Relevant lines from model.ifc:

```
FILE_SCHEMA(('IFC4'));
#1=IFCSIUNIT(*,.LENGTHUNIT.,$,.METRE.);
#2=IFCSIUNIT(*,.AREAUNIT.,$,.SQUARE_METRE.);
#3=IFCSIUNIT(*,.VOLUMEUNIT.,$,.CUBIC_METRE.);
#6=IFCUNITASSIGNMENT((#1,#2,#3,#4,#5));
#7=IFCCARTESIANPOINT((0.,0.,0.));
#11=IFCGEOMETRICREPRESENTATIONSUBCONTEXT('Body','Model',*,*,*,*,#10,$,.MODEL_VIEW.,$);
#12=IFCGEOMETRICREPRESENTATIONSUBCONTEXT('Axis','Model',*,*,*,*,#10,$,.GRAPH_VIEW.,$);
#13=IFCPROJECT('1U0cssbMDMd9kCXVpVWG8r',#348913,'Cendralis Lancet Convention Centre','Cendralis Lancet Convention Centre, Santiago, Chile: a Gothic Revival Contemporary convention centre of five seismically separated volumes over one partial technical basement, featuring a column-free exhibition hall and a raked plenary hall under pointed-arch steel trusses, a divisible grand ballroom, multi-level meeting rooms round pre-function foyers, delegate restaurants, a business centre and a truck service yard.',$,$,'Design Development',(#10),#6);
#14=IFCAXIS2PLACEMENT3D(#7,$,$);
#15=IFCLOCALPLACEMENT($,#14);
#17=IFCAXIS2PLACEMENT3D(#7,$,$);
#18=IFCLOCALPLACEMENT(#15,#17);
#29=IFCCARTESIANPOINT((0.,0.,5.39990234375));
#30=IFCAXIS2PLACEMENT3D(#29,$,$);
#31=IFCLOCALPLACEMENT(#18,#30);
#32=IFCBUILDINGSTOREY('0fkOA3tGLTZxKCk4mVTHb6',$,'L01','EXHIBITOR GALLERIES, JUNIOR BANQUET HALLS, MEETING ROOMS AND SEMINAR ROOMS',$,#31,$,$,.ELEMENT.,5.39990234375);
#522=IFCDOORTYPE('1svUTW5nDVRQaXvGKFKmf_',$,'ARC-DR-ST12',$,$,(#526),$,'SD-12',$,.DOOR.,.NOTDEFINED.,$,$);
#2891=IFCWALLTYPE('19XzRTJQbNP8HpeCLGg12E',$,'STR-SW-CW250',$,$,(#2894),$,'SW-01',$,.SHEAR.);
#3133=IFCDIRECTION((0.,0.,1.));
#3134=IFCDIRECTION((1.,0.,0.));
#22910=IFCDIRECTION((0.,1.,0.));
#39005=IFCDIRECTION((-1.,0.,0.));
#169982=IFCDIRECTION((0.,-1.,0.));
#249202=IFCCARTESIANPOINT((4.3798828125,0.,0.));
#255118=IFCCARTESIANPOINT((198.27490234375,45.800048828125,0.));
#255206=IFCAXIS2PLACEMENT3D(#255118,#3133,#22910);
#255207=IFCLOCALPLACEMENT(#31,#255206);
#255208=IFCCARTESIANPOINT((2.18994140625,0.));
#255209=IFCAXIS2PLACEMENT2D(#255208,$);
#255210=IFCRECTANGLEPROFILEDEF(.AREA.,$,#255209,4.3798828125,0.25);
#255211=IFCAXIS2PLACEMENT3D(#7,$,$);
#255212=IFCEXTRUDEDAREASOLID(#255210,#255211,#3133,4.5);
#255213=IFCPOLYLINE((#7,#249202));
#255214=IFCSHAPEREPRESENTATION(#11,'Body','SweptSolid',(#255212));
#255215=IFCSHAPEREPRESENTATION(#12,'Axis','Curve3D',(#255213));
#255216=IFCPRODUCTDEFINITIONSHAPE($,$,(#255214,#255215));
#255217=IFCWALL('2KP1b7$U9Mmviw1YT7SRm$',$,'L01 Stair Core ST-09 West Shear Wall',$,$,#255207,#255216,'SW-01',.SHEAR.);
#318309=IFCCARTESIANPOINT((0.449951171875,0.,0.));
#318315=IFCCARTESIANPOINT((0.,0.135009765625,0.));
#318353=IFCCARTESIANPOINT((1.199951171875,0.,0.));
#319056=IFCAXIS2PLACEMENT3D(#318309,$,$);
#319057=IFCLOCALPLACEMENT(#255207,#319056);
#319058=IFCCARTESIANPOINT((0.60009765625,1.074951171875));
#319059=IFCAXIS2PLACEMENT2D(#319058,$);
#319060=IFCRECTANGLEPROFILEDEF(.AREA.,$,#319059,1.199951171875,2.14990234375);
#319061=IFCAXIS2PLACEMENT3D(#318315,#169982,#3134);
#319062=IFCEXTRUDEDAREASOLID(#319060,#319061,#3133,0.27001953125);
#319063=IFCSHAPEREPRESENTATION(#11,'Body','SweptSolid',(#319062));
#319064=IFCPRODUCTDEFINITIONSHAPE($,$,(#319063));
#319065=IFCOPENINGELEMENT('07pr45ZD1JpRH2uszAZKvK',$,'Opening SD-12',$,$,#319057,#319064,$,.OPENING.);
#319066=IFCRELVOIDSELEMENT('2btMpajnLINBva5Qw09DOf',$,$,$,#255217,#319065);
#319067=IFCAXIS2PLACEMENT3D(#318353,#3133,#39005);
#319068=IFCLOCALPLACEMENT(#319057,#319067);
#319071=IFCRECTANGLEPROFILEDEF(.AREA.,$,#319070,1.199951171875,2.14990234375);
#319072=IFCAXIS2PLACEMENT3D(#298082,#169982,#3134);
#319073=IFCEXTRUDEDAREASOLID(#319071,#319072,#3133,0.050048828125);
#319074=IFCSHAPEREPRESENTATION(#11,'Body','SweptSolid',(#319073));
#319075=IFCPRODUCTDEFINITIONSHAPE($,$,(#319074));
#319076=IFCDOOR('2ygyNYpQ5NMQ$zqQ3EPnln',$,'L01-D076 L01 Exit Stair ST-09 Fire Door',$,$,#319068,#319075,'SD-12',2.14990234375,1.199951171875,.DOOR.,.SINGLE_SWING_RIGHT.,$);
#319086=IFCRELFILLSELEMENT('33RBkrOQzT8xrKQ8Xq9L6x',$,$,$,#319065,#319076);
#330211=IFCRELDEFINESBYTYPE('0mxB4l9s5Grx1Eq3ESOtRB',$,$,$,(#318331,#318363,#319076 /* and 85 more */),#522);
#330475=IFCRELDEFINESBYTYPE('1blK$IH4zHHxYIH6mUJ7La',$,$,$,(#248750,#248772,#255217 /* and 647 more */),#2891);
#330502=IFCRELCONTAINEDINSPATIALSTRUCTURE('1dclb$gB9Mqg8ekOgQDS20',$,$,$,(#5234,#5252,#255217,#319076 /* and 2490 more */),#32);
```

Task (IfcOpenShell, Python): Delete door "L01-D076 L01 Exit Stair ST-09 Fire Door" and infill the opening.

```python
import ifcopenshell
import ifcopenshell.api.feature
import ifcopenshell.api.root
import ifcopenshell.geom
import ifcopenshell.util.shape

model = ifcopenshell.open("model.ifc")
settings = ifcopenshell.geom.settings()


def volume(element):
    """Net volume in cubic metres, openings subtracted."""
    shape = ifcopenshell.geom.create_shape(settings, element)
    return ifcopenshell.util.shape.get_volume(shape.geometry)


door = model.by_guid("2ygyNYpQ5NMQ$zqQ3EPnln")
opening = door.FillsVoids[0].RelatingOpeningElement
wall = opening.VoidsElements[0].RelatingBuildingElement
before = volume(wall)

ifcopenshell.api.root.remove_product(model, product=door)
ifcopenshell.api.feature.remove_feature(model, feature=opening)

after = volume(wall)

print(f"wall volume {before:.3f} -> {after:.3f} m3")

model.write("model-out.ifc")
```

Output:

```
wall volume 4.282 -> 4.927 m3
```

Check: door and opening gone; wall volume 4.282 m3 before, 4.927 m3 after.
